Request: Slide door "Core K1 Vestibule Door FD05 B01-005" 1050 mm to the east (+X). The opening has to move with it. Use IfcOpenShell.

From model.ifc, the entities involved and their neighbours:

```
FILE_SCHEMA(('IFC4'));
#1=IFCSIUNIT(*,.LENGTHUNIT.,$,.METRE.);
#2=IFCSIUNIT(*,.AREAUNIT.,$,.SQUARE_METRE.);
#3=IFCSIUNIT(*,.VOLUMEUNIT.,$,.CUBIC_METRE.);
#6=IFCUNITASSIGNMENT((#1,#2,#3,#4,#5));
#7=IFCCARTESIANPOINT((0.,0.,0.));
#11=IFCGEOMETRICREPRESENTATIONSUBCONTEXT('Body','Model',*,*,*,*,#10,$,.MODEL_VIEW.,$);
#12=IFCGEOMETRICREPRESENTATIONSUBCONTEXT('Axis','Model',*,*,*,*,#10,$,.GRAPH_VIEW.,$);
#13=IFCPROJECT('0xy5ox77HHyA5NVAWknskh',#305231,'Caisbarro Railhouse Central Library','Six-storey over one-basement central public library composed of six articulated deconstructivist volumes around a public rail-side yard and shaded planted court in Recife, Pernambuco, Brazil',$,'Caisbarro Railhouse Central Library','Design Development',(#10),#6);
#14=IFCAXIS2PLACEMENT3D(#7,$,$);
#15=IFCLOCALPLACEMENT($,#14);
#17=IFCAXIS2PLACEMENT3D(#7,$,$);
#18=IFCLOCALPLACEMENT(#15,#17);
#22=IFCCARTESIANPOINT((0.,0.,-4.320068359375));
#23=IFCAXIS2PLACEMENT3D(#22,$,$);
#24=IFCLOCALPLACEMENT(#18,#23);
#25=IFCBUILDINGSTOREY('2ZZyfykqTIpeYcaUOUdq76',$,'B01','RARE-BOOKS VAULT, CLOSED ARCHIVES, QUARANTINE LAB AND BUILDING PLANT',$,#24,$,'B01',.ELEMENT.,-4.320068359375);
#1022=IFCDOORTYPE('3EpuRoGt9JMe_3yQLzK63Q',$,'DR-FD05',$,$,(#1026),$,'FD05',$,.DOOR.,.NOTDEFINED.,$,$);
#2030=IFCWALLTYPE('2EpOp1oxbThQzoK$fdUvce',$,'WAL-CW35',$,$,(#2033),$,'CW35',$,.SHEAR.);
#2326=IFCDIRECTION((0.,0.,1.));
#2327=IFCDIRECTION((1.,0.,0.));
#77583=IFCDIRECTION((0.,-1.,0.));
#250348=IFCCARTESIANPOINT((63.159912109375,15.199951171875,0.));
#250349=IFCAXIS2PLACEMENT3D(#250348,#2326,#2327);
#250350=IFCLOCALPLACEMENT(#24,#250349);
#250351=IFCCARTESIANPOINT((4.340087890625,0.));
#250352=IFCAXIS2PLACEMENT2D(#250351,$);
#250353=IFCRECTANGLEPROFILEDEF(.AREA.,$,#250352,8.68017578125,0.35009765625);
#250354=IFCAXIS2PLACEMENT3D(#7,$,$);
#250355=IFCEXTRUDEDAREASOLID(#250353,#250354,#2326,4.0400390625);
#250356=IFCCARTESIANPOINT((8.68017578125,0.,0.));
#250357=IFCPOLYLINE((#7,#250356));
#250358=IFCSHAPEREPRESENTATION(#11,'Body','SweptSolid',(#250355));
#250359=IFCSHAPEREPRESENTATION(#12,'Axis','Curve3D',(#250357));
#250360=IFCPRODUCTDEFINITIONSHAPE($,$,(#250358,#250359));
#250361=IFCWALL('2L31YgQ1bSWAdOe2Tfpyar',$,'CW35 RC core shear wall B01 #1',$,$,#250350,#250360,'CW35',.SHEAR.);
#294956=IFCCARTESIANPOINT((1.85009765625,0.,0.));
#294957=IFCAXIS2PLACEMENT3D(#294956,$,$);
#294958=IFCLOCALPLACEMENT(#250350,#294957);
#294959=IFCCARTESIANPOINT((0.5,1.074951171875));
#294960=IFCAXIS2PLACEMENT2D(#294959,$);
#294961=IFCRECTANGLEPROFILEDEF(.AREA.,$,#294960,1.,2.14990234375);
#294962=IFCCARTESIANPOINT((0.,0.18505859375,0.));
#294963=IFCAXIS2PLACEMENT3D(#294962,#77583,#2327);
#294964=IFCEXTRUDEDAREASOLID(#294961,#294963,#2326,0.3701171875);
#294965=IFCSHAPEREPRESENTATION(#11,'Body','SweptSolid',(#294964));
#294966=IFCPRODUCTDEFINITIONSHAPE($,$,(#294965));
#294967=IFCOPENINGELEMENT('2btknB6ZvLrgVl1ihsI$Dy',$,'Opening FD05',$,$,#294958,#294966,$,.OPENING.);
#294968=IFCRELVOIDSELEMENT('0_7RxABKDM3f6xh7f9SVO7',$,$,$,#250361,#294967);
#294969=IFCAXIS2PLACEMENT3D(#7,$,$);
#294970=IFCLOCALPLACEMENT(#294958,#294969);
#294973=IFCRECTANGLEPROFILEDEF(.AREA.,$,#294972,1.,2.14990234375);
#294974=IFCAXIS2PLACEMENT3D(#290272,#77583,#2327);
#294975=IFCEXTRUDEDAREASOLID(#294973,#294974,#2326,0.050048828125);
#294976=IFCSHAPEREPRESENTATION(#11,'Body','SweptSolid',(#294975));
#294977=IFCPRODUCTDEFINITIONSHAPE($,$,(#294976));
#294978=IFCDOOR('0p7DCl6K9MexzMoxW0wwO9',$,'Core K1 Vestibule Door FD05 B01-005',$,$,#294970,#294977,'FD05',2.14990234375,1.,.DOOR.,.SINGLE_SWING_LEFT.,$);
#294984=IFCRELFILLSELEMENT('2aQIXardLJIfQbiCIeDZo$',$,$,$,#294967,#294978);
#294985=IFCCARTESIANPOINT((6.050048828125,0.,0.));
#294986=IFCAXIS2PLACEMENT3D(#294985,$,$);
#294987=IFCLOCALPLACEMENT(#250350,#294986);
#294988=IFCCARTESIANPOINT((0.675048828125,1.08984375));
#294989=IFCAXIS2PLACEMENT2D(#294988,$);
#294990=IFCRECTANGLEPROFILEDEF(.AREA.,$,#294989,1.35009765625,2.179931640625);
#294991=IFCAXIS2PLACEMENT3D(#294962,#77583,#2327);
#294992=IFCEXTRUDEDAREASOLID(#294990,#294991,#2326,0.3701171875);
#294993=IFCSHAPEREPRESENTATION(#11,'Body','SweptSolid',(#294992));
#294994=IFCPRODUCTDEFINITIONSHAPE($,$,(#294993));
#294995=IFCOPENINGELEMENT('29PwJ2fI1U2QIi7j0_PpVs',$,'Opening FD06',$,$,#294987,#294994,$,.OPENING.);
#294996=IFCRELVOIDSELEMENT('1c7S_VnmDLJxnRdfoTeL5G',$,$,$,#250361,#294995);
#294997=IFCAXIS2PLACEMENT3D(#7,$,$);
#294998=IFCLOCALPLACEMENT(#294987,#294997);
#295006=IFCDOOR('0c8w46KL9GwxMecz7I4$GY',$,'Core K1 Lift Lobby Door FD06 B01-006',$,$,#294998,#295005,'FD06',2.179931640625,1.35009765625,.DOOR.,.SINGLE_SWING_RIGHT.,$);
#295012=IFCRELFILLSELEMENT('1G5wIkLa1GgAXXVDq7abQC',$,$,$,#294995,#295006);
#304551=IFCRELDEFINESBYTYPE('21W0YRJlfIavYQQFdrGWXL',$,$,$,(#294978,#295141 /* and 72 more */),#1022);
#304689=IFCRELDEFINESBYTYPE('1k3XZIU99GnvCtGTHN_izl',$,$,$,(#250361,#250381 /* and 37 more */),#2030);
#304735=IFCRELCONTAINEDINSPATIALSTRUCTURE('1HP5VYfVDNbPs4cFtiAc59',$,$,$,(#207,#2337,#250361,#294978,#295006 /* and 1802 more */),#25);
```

```python
import ifcopenshell
import ifcopenshell.api.geometry
import ifcopenshell.util.placement
import ifcopenshell.util.unit

model = ifcopenshell.open("model.ifc")
unit_scale = ifcopenshell.util.unit.calculate_unit_scale(model)

door = model.by_guid("0p7DCl6K9MexzMoxW0wwO9")
opening = door.FillsVoids[0].RelatingOpeningElement
wall = opening.VoidsElements[0].RelatingBuildingElement

wall_matrix = ifcopenshell.util.placement.get_local_placement(wall.ObjectPlacement)
shift = wall_matrix[:3, 0] * 1.05 / unit_scale
before = ifcopenshell.util.placement.get_local_placement(door.ObjectPlacement)[:3, 3].copy()

# The door is placed relative to its opening, so it follows when the opening moves.
matrix = ifcopenshell.util.placement.get_local_placement(opening.ObjectPlacement)
matrix[:3, 3] += shift
ifcopenshell.api.geometry.edit_object_placement(
    model, product=opening, matrix=matrix, is_si=False, should_transform_children=True
)

after = ifcopenshell.util.placement.get_local_placement(door.ObjectPlacement)[:3, 3]
print("door moved by", (after - before).round(3) + 0.0)

model.write("model_v2.ifc")
```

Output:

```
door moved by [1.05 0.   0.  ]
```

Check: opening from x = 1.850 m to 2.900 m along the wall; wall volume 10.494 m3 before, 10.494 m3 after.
